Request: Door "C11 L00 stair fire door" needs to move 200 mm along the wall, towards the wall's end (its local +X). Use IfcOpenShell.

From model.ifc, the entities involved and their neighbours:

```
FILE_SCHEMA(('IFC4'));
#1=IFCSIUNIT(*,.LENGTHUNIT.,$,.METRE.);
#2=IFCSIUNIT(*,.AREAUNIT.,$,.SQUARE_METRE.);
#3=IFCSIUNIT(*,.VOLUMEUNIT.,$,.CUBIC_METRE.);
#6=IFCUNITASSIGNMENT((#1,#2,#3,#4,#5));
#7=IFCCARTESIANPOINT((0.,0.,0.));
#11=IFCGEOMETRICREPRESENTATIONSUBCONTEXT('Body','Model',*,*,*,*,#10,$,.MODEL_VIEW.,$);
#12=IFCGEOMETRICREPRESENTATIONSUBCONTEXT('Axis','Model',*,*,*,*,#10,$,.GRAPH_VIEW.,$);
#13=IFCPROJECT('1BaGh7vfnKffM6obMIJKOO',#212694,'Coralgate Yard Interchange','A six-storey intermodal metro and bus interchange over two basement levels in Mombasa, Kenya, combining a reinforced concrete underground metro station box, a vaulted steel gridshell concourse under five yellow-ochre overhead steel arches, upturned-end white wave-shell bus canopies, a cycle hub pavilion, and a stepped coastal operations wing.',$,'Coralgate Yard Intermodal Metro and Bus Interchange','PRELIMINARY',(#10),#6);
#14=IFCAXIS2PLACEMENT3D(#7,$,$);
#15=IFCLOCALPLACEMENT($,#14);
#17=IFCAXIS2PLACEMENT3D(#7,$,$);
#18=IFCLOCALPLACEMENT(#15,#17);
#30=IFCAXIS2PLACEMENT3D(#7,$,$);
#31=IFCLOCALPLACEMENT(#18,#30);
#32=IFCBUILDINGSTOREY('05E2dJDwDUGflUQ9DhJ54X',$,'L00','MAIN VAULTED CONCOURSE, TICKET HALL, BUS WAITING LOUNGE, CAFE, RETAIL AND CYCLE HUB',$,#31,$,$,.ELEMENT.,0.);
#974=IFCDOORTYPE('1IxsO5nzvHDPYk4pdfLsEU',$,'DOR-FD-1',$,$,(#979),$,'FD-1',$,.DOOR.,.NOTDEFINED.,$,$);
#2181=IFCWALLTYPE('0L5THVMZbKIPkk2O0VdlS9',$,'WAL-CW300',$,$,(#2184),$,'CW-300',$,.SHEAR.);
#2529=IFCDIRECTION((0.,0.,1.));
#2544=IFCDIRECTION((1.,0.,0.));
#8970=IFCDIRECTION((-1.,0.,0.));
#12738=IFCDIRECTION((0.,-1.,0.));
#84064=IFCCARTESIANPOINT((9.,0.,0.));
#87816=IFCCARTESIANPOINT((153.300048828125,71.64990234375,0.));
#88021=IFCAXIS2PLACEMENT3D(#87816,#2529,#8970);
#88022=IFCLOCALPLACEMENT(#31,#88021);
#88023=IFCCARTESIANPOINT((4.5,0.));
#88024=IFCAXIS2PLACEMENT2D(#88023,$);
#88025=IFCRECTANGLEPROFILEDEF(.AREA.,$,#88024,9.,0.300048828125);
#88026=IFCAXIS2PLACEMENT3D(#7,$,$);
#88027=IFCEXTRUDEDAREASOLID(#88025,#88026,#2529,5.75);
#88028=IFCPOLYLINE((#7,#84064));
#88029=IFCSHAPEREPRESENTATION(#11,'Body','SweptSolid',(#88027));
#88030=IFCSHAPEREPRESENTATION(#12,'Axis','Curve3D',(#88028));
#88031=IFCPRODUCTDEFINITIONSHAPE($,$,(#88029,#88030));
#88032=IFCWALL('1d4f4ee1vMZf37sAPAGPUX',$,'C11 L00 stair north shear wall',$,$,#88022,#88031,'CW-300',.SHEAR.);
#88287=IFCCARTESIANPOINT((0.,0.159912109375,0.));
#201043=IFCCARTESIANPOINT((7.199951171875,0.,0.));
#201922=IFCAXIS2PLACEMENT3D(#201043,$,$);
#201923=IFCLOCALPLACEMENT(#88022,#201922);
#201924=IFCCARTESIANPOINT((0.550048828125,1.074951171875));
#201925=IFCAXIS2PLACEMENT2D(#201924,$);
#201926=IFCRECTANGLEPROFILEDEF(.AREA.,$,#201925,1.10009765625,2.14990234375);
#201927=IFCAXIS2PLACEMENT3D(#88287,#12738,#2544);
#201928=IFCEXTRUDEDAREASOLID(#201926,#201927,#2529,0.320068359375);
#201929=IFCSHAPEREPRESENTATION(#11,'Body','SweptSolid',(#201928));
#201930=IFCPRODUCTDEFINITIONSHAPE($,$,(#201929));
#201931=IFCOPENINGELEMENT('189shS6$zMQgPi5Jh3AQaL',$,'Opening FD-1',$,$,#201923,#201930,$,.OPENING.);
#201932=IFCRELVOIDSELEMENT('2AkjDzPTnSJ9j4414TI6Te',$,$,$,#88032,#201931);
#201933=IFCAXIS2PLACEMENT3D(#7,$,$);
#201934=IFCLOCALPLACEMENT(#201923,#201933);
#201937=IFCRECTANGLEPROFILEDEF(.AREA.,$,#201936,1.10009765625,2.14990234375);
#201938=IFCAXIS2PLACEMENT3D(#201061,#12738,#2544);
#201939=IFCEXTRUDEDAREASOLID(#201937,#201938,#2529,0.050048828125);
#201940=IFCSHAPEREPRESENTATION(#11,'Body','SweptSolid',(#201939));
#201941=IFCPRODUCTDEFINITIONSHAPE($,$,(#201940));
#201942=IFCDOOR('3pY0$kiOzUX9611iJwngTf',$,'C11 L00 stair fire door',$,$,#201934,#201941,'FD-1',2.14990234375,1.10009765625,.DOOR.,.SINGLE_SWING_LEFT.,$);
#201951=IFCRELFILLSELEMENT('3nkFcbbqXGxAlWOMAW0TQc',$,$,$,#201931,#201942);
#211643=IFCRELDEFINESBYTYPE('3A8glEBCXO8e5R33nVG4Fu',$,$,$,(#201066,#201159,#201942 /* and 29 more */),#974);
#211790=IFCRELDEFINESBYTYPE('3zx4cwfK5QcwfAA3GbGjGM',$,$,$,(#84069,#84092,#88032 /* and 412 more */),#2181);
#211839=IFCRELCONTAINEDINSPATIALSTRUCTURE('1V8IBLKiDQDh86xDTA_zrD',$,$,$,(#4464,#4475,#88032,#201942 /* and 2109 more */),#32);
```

```python
import ifcopenshell
import ifcopenshell.api.geometry
import ifcopenshell.util.placement

model = ifcopenshell.open("model.ifc")

door = model.by_guid("3pY0$kiOzUX9611iJwngTf")
opening = door.FillsVoids[0].RelatingOpeningElement
wall = opening.VoidsElements[0].RelatingBuildingElement

wall_matrix = ifcopenshell.util.placement.get_local_placement(wall.ObjectPlacement)
shift = wall_matrix[:3, 0] * 0.2
before = ifcopenshell.util.placement.get_local_placement(door.ObjectPlacement)[:3, 3].copy()

# The door is placed relative to its opening, so it follows when the opening moves.
matrix = ifcopenshell.util.placement.get_local_placement(opening.ObjectPlacement)
matrix[:3, 3] += shift
ifcopenshell.api.geometry.edit_object_placement(
    model, product=opening, matrix=matrix, is_si=False, should_transform_children=True
)

after = ifcopenshell.util.placement.get_local_placement(door.ObjectPlacement)[:3, 3]
print("door moved by", (after - before).round(3) + 0.0)

model.write("model_updated.ifc")
```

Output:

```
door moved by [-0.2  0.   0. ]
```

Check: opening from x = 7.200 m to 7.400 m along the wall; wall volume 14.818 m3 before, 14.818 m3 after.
